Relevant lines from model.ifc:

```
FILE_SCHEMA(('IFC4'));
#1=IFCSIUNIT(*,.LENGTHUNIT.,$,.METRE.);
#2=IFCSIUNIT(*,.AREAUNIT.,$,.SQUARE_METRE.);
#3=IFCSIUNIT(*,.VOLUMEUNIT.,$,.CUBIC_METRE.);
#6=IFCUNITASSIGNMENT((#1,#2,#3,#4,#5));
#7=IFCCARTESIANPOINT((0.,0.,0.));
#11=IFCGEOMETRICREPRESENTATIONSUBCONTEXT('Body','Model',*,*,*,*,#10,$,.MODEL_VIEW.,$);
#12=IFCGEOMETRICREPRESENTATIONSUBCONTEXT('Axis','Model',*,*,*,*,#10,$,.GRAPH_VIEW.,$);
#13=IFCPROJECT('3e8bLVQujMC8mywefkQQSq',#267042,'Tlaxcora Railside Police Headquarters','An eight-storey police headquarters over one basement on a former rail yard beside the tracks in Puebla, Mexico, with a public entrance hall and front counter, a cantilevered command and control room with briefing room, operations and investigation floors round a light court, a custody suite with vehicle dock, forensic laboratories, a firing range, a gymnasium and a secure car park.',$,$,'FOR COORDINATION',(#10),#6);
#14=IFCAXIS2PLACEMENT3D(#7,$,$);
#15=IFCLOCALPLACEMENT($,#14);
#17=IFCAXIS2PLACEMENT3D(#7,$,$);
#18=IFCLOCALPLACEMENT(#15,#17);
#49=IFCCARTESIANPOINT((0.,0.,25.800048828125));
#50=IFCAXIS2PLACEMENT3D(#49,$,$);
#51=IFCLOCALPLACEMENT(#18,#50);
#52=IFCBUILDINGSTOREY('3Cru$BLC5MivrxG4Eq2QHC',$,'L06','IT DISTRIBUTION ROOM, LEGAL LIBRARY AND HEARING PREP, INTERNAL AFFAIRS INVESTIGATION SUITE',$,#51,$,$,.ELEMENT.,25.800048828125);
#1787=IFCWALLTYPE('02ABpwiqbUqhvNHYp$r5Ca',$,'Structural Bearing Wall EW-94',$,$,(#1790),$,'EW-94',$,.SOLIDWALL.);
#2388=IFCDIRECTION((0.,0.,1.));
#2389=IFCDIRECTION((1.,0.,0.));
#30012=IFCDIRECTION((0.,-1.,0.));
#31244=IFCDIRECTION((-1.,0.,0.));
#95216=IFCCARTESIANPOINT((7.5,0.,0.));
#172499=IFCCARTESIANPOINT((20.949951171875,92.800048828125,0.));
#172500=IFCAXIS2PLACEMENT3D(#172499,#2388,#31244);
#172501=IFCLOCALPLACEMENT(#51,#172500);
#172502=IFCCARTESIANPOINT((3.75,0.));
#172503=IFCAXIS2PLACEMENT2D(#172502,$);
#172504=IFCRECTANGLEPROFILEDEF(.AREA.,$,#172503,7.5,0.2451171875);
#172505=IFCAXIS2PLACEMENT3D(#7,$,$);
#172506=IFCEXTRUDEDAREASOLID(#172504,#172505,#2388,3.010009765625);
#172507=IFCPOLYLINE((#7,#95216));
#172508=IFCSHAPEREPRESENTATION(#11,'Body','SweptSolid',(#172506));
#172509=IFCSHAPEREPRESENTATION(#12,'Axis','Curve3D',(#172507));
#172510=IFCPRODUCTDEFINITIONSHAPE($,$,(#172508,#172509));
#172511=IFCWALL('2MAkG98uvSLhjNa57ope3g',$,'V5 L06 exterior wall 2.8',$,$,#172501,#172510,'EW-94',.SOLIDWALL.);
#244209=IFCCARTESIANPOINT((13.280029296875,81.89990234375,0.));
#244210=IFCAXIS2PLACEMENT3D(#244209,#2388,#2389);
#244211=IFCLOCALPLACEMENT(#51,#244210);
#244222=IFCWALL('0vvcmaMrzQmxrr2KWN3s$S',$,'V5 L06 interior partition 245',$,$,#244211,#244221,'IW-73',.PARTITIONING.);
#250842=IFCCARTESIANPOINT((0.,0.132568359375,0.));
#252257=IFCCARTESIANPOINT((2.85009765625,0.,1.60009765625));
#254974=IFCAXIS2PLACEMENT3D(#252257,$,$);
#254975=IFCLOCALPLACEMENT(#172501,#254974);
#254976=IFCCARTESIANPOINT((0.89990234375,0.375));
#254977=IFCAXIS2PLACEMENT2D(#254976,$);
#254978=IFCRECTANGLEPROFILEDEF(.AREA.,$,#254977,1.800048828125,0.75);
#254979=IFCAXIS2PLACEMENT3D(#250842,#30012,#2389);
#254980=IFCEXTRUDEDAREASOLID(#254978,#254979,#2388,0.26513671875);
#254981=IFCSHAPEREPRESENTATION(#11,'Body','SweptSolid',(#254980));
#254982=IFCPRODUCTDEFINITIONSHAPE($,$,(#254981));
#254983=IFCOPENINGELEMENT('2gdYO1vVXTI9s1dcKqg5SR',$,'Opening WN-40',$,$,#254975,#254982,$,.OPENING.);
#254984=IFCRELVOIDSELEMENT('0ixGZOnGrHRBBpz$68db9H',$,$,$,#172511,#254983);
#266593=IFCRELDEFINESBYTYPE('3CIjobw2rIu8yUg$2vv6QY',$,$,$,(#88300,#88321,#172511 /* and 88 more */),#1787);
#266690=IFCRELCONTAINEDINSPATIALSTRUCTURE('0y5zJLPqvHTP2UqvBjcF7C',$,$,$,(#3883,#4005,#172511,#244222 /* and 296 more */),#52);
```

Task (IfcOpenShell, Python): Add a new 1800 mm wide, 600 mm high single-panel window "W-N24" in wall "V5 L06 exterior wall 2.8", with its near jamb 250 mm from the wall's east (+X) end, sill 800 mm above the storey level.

```python
import numpy as np
import ifcopenshell
import ifcopenshell.api.feature
import ifcopenshell.api.geometry
import ifcopenshell.api.root
import ifcopenshell.api.spatial
import ifcopenshell.geom
import ifcopenshell.util.element
import ifcopenshell.util.placement
import ifcopenshell.util.representation
import ifcopenshell.util.shape
import ifcopenshell.util.unit

model = ifcopenshell.open("model.ifc")
unit_scale = ifcopenshell.util.unit.calculate_unit_scale(model)
settings = ifcopenshell.geom.settings()


def volume(element):
    """Net volume in cubic metres, openings subtracted."""
    shape = ifcopenshell.geom.create_shape(settings, element)
    return ifcopenshell.util.shape.get_volume(shape.geometry)


wall = model.by_id(172511)
storey = ifcopenshell.util.element.get_container(wall, ifc_class="IfcBuildingStorey")
context = ifcopenshell.util.representation.get_context(model, "Model", "Body", "MODEL_VIEW")
before = volume(wall)

width, height, from_end, sill = 1.8, 0.6, 0.25, 0.8  # metres

# The wall runs along its own X axis, and the end named is its -X end.
wall_shape = ifcopenshell.geom.create_shape(settings, wall)
x, y, z = ifcopenshell.util.shape.get_vertices(wall_shape.geometry).T
start = x.min() + from_end
face, thickness = float(y.min()), float(y.max() - y.min())
wall_matrix = ifcopenshell.util.placement.get_local_placement(wall.ObjectPlacement)
level = ifcopenshell.util.placement.get_local_placement(storey.ObjectPlacement)[2, 3]


def in_wall(x, y):
    """Placement at x, y metres in the wall's axes, at sill height."""
    matrix = wall_matrix.copy()
    matrix[:, 3] = wall_matrix @ np.array([x / unit_scale, y / unit_scale, 0.0, 1.0])
    matrix[2, 3] = level + sill / unit_scale
    return matrix


# Opening: a box that overshoots both wall faces by 50 mm.
opening = ifcopenshell.api.root.create_entity(model, ifc_class="IfcOpeningElement", predefined_type="OPENING")
box = ifcopenshell.api.geometry.add_wall_representation(
    model, context=context, length=width, height=height, thickness=thickness + 0.1
)
ifcopenshell.api.geometry.assign_representation(model, product=opening, representation=box)
ifcopenshell.api.geometry.edit_object_placement(model, product=opening, matrix=in_wall(start, face - 0.05), is_si=False)
ifcopenshell.api.feature.add_feature(model, feature=opening, element=wall)

window = ifcopenshell.api.root.create_entity(model, ifc_class="IfcWindow", name="W-N24", predefined_type="WINDOW")
window.OverallWidth, window.OverallHeight = width / unit_scale, height / unit_scale
window.PartitioningType = "SINGLE_PANEL"
body = ifcopenshell.api.geometry.add_window_representation(
    model,
    context=context,
    overall_width=window.OverallWidth,
    overall_height=window.OverallHeight,
    partition_type="SINGLE_PANEL",
)
ifcopenshell.api.geometry.assign_representation(model, product=window, representation=body)
ifcopenshell.api.spatial.assign_container(model, products=[window], relating_structure=storey)
ifcopenshell.api.feature.add_filling(model, opening=opening, element=window)

# Centre the window in the wall's thickness.
ifcopenshell.api.geometry.edit_object_placement(model, product=window, matrix=in_wall(start, face), is_si=False)
window_shape = ifcopenshell.geom.create_shape(settings, window)
depth = ifcopenshell.util.shape.get_vertices(window_shape.geometry)[:, 1]
offset = face + thickness / 2 - (depth.min() + depth.max()) / 2
ifcopenshell.api.geometry.edit_object_placement(model, product=window, matrix=in_wall(start, offset), is_si=False)

after = volume(wall)

print(f"wall volume {before:.3f} -> {after:.3f} m3")

model.write("model_rev.ifc")
```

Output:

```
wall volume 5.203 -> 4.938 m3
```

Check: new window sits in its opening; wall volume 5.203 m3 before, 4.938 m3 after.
